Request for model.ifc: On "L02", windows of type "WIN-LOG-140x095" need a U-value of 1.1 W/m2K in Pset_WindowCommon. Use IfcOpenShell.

First a look at what the model holds.

```python
import ifcopenshell
import ifcopenshell.util.element

model = ifcopenshell.open("model.ifc")
print(model.schema)
storey = next(s for s in model.by_type("IfcBuildingStorey") if s.Name == "L02")
windows = [e for e in ifcopenshell.util.element.get_decomposition(storey) if e.is_a("IfcWindow")]
seen = {}
for e in windows:
    element_type = ifcopenshell.util.element.get_type(e)
    key = (element_type.Name if element_type != e and element_type else None, ifcopenshell.util.element.get_pset(e, "Pset_WindowCommon", "ThermalTransmittance"))
    seen[key] = seen.get(key, 0) + 1
for (name, value), count in sorted(seen.items(), key=str):
    print(count, "x", name, "|", value)
```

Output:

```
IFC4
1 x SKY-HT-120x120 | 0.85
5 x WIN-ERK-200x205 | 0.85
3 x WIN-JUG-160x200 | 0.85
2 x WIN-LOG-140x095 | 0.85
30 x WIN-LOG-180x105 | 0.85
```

```python
import ifcopenshell
import ifcopenshell.api.pset
import ifcopenshell.util.element

model = ifcopenshell.open("model.ifc")

storey = next(s for s in model.by_type("IfcBuildingStorey") if s.Name == "L02")
windows = [e for e in ifcopenshell.util.element.get_decomposition(storey) if e.is_a("IfcWindow")]

count = 0
for e in windows:
    element_type = ifcopenshell.util.element.get_type(e)
    if element_type in (None, e) or element_type.Name != "WIN-LOG-140x095":
        continue
    # add_pset returns the element's existing set when there is one.
    pset = ifcopenshell.api.pset.add_pset(model, product=e, name="Pset_WindowCommon")
    ifcopenshell.api.pset.edit_pset(model, pset=pset, properties={"ThermalTransmittance": 1.1})
    count += 1

print(count, "windows updated")

model.write("model_updated.ifc")
```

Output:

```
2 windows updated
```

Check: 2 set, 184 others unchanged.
